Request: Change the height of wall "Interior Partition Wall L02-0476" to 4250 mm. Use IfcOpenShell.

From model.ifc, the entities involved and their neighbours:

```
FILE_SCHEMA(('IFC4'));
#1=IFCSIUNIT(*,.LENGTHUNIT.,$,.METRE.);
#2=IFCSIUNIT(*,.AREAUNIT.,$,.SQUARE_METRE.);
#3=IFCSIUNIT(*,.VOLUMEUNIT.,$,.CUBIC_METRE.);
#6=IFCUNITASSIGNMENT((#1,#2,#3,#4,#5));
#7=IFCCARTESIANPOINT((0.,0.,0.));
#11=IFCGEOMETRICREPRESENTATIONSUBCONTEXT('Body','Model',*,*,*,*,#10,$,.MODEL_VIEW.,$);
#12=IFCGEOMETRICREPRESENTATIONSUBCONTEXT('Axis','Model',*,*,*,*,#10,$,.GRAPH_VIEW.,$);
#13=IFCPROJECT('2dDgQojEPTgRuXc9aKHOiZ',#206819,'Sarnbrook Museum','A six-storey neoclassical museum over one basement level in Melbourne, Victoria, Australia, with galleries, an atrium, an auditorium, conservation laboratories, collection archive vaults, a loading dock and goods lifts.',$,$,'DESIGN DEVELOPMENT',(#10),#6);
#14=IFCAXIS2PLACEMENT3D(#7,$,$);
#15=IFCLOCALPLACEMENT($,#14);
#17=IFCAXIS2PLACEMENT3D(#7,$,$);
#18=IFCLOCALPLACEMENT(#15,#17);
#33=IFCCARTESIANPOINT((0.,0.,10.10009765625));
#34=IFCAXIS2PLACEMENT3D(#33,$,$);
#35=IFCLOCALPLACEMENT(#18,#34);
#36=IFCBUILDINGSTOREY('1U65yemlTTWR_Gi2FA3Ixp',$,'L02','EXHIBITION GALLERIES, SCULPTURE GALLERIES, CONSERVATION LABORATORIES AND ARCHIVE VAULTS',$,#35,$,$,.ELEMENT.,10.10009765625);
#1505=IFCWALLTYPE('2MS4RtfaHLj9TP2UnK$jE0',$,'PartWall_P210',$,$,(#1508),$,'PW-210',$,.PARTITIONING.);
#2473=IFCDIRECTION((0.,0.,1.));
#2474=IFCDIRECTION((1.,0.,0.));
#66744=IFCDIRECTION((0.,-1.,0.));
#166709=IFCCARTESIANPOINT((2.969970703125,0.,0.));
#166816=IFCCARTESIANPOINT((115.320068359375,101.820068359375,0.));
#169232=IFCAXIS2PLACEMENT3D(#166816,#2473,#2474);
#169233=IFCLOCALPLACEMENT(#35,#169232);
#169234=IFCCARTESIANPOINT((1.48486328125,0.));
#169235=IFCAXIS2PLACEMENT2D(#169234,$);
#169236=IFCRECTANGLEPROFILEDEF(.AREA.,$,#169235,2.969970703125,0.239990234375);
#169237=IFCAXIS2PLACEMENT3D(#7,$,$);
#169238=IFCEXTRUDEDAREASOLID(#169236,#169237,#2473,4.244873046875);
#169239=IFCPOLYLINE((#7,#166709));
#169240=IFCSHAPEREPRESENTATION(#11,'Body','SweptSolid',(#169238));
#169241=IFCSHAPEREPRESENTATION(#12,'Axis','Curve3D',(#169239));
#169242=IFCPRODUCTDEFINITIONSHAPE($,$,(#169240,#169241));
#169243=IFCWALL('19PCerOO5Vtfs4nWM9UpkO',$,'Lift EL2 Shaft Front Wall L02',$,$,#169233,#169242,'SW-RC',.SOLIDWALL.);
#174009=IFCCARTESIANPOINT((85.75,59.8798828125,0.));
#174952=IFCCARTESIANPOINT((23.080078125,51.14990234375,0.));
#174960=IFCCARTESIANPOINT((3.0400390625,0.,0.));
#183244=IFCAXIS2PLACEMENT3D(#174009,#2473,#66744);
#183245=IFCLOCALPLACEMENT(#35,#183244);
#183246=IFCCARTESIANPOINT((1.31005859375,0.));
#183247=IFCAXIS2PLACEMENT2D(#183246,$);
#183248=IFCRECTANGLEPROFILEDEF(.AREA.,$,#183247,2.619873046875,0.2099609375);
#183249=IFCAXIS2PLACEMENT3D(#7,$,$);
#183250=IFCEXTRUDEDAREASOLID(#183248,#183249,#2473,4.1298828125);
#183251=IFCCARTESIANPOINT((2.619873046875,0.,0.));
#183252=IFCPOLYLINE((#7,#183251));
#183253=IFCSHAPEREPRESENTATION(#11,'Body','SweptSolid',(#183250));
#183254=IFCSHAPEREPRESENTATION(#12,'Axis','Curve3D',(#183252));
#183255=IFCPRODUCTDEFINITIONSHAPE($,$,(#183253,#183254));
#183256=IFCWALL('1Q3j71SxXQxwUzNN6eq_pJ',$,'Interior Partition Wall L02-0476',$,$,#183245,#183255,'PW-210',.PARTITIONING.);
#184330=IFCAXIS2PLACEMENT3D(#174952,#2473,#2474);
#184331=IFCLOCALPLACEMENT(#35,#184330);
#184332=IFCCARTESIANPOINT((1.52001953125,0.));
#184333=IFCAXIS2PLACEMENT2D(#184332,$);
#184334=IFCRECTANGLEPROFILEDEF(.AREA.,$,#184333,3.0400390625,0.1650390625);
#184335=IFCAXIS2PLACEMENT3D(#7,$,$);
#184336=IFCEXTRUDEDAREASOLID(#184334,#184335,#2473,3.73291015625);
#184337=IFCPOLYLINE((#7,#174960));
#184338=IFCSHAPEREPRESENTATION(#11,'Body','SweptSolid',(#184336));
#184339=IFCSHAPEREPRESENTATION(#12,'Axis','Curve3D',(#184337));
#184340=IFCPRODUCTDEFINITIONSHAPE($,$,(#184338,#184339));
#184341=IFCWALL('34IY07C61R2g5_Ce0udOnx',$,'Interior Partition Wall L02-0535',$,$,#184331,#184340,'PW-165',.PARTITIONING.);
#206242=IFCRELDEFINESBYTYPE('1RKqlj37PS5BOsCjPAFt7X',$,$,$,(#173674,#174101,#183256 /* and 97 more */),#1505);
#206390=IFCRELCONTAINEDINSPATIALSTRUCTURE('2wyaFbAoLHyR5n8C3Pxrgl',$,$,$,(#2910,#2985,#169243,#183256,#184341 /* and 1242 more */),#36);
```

```python
import ifcopenshell
import ifcopenshell.geom
import ifcopenshell.util.representation
import ifcopenshell.util.shape
import ifcopenshell.util.unit

model = ifcopenshell.open("model.ifc")
unit_scale = ifcopenshell.util.unit.calculate_unit_scale(model)
settings = ifcopenshell.geom.settings()


def volume(element):
    """Net volume in cubic metres, openings subtracted."""
    shape = ifcopenshell.geom.create_shape(settings, element)
    return ifcopenshell.util.shape.get_volume(shape.geometry)


wall = model.by_guid("1Q3j71SxXQxwUzNN6eq_pJ")
before = volume(wall)

body = ifcopenshell.util.representation.get_representation(wall, "Model", "Body")
solid = body.Items[0]
old_height = solid.Depth
solid.Depth = 4.25 / unit_scale
after = volume(wall)

print(f"height {old_height:g} -> {solid.Depth:g}, volume {before:.3f} -> {after:.3f} m3")

model.write("model-out.ifc")
```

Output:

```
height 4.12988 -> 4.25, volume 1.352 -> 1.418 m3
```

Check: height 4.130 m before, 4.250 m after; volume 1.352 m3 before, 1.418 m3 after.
